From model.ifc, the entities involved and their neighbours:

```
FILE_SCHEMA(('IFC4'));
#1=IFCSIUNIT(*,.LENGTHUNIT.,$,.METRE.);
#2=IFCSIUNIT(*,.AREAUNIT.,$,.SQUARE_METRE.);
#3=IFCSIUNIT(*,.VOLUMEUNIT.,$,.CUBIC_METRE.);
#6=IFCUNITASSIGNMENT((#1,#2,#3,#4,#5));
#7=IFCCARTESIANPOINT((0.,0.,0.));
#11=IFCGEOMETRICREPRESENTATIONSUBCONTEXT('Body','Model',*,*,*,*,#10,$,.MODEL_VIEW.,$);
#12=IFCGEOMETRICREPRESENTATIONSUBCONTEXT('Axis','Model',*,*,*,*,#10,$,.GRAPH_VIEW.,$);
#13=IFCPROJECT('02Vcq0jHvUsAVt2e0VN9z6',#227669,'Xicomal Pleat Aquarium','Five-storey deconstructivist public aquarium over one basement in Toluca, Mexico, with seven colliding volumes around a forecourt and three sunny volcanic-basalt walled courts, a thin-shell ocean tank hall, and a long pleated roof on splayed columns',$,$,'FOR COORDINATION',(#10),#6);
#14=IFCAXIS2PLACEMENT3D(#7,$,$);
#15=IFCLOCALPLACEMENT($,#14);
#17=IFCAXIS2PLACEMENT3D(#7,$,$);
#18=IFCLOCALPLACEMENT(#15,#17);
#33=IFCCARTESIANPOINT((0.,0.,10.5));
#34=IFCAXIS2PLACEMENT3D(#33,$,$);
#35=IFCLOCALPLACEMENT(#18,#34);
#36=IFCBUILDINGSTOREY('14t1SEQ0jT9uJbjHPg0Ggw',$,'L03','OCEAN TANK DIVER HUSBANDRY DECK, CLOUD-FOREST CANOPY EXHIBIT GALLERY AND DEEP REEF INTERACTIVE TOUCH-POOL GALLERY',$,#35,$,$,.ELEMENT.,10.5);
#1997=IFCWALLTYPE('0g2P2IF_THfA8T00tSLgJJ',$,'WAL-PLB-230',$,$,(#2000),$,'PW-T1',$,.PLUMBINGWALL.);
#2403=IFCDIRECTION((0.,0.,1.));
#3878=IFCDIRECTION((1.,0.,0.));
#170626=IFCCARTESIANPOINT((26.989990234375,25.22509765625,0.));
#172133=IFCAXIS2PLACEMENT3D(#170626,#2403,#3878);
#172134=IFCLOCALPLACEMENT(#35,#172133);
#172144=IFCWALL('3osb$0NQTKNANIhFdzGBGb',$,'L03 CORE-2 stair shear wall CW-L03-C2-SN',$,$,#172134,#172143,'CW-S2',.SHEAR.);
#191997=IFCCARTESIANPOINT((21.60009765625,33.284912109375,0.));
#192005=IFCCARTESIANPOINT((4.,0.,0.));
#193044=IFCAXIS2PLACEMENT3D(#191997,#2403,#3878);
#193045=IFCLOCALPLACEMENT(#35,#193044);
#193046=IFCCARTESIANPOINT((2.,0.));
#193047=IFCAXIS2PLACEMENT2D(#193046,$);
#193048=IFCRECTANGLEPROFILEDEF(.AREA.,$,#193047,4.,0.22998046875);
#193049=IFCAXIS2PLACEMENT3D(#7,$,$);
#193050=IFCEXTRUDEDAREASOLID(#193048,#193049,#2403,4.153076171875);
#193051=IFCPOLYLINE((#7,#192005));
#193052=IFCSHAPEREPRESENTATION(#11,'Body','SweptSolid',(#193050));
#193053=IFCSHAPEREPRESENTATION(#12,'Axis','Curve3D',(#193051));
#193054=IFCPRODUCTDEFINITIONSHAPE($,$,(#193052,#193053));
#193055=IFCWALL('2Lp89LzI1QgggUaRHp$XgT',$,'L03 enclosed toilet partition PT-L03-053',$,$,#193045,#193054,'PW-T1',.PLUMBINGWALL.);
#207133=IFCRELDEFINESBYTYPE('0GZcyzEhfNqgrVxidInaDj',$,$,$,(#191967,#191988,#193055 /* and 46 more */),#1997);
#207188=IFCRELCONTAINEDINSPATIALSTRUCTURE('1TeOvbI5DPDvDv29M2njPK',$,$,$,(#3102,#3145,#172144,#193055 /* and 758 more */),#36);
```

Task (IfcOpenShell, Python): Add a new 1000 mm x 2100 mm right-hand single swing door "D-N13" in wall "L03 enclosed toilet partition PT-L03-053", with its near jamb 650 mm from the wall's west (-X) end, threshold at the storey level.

```python
import numpy as np
import ifcopenshell
import ifcopenshell.api.feature
import ifcopenshell.api.geometry
import ifcopenshell.api.root
import ifcopenshell.api.spatial
import ifcopenshell.geom
import ifcopenshell.util.element
import ifcopenshell.util.placement
import ifcopenshell.util.representation
import ifcopenshell.util.shape
import ifcopenshell.util.unit

model = ifcopenshell.open("model.ifc")
unit_scale = ifcopenshell.util.unit.calculate_unit_scale(model)
settings = ifcopenshell.geom.settings()


def volume(element):
    """Net volume in cubic metres, openings subtracted."""
    shape = ifcopenshell.geom.create_shape(settings, element)
    return ifcopenshell.util.shape.get_volume(shape.geometry)


wall = model.by_guid("2Lp89LzI1QgggUaRHp$XgT")
storey = ifcopenshell.util.element.get_container(wall, ifc_class="IfcBuildingStorey")
context = ifcopenshell.util.representation.get_context(model, "Model", "Body", "MODEL_VIEW")
before = volume(wall)

width, height, from_end, sill = 1, 2.1, 0.65, 0.0  # metres

# The wall runs along its own X axis, and the end named is its -X end.
wall_shape = ifcopenshell.geom.create_shape(settings, wall)
x, y, z = ifcopenshell.util.shape.get_vertices(wall_shape.geometry).T
start = x.min() + from_end
face, thickness = float(y.min()), float(y.max() - y.min())
wall_matrix = ifcopenshell.util.placement.get_local_placement(wall.ObjectPlacement)
level = ifcopenshell.util.placement.get_local_placement(storey.ObjectPlacement)[2, 3]


def in_wall(x, y):
    """Placement at x, y metres in the wall's axes, at sill height."""
    matrix = wall_matrix.copy()
    matrix[:, 3] = wall_matrix @ np.array([x / unit_scale, y / unit_scale, 0.0, 1.0])
    matrix[2, 3] = level + sill / unit_scale
    return matrix


# Opening: a box that overshoots both wall faces by 50 mm.
opening = ifcopenshell.api.root.create_entity(model, ifc_class="IfcOpeningElement", predefined_type="OPENING")
box = ifcopenshell.api.geometry.add_wall_representation(
    model, context=context, length=width, height=height, thickness=thickness + 0.1
)
ifcopenshell.api.geometry.assign_representation(model, product=opening, representation=box)
ifcopenshell.api.geometry.edit_object_placement(model, product=opening, matrix=in_wall(start, face - 0.05), is_si=False)
ifcopenshell.api.feature.add_feature(model, feature=opening, element=wall)

door = ifcopenshell.api.root.create_entity(model, ifc_class="IfcDoor", name="D-N13", predefined_type="DOOR")
door.OverallWidth, door.OverallHeight = width / unit_scale, height / unit_scale
door.OperationType = "SINGLE_SWING_RIGHT"
body = ifcopenshell.api.geometry.add_door_representation(
    model,
    context=context,
    overall_width=door.OverallWidth,
    overall_height=door.OverallHeight,
    operation_type="SINGLE_SWING_RIGHT",
    lining_properties={"LiningDepth": thickness / unit_scale, "ThresholdDepth": thickness / unit_scale},
)
ifcopenshell.api.geometry.assign_representation(model, product=door, representation=body)
ifcopenshell.api.spatial.assign_container(model, products=[door], relating_structure=storey)
ifcopenshell.api.feature.add_filling(model, opening=opening, element=door)

# The lining spans the wall, so the door starts at the wall face.
ifcopenshell.api.geometry.edit_object_placement(model, product=door, matrix=in_wall(start, face), is_si=False)

after = volume(wall)

print(f"wall volume {before:.3f} -> {after:.3f} m3")

model.write("model_updated.ifc")
```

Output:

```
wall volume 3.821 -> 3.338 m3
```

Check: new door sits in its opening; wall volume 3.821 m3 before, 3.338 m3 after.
